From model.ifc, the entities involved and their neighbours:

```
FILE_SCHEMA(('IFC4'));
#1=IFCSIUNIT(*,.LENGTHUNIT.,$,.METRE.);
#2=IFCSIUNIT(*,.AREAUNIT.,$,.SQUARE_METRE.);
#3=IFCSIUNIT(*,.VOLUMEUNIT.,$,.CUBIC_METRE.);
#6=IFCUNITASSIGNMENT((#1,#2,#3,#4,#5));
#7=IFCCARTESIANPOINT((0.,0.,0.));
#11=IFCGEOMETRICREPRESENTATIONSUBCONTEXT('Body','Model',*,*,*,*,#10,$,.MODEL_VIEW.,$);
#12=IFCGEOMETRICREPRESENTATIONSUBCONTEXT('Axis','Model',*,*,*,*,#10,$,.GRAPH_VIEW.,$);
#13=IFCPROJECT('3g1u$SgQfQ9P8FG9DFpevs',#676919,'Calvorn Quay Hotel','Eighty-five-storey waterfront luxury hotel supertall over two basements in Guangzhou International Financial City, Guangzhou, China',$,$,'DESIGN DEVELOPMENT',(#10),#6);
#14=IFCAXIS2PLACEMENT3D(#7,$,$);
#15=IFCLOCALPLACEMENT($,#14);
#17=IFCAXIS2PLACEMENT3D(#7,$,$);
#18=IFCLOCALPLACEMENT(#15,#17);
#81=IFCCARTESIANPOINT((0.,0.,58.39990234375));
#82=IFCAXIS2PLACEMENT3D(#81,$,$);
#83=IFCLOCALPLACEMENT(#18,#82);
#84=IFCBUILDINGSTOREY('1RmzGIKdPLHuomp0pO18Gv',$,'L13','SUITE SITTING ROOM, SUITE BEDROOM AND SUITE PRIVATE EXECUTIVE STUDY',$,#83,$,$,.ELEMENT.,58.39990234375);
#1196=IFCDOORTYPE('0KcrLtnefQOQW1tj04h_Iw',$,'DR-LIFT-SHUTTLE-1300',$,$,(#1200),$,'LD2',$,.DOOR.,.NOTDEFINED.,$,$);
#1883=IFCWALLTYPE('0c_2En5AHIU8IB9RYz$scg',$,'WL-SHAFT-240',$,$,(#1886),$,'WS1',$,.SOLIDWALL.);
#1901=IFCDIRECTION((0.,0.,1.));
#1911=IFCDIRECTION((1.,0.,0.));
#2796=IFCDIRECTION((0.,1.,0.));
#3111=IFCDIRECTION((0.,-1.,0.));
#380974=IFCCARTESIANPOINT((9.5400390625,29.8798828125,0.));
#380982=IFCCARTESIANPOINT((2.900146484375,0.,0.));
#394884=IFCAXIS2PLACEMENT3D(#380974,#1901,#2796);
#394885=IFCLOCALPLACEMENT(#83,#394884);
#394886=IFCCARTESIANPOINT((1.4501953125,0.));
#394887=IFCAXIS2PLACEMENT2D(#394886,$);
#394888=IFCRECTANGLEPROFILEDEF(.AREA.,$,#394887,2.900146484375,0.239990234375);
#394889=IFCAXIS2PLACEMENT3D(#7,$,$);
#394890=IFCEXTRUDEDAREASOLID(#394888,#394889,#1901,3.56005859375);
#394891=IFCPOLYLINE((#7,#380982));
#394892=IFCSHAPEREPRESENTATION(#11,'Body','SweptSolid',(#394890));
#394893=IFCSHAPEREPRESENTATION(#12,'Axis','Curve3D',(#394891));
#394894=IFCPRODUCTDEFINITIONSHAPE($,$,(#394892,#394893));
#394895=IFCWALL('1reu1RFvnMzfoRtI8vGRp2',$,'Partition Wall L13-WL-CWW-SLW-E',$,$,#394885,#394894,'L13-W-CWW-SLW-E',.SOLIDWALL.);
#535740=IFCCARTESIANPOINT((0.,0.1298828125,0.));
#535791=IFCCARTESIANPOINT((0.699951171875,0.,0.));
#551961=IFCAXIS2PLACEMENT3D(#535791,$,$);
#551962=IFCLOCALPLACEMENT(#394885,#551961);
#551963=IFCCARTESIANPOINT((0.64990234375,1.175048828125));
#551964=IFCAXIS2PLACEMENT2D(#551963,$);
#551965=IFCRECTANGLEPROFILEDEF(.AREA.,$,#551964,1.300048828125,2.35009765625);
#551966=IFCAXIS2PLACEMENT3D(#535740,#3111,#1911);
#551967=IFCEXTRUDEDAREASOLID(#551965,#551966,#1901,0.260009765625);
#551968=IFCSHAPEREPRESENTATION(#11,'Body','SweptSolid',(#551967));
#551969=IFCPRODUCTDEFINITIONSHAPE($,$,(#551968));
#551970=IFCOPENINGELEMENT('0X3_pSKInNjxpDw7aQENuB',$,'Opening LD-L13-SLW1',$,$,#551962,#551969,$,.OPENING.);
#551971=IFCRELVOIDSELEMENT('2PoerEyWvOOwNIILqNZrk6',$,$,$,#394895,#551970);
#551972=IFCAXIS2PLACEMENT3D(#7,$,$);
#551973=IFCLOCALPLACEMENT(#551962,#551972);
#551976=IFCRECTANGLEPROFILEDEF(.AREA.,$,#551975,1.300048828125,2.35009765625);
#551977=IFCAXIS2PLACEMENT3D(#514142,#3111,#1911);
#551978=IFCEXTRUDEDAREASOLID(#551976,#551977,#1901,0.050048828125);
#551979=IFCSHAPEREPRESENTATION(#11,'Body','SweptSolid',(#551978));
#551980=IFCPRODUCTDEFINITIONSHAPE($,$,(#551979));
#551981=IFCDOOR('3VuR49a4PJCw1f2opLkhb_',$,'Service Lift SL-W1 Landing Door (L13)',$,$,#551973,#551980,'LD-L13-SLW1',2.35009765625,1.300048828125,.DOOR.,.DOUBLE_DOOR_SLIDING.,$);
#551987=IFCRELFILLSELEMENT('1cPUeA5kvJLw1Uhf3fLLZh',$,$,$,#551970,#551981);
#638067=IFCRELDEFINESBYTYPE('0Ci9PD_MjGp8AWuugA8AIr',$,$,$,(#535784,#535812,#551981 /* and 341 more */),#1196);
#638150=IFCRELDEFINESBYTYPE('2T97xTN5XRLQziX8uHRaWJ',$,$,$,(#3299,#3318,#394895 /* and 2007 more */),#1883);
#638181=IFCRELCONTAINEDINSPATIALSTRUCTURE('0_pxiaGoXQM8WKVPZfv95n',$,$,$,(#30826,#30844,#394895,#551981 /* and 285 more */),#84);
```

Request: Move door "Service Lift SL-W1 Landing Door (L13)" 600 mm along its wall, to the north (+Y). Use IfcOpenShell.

```python
import ifcopenshell
import ifcopenshell.api.geometry
import ifcopenshell.util.placement
import ifcopenshell.util.unit

model = ifcopenshell.open("model.ifc")
unit_scale = ifcopenshell.util.unit.calculate_unit_scale(model)

door = model.by_id(551981)
opening = door.FillsVoids[0].RelatingOpeningElement
wall = opening.VoidsElements[0].RelatingBuildingElement

wall_matrix = ifcopenshell.util.placement.get_local_placement(wall.ObjectPlacement)
shift = wall_matrix[:3, 0] * 0.6 / unit_scale
before = ifcopenshell.util.placement.get_local_placement(door.ObjectPlacement)[:3, 3].copy()

# The door is placed relative to its opening, so it follows when the opening moves.
matrix = ifcopenshell.util.placement.get_local_placement(opening.ObjectPlacement)
matrix[:3, 3] += shift
ifcopenshell.api.geometry.edit_object_placement(
    model, product=opening, matrix=matrix, is_si=False, should_transform_children=True
)

after = ifcopenshell.util.placement.get_local_placement(door.ObjectPlacement)[:3, 3]
print("door moved by", (after - before).round(3) + 0.0)

model.write("model_v2.ifc")
```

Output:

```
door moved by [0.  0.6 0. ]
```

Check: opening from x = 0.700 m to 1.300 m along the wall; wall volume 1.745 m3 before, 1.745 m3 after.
